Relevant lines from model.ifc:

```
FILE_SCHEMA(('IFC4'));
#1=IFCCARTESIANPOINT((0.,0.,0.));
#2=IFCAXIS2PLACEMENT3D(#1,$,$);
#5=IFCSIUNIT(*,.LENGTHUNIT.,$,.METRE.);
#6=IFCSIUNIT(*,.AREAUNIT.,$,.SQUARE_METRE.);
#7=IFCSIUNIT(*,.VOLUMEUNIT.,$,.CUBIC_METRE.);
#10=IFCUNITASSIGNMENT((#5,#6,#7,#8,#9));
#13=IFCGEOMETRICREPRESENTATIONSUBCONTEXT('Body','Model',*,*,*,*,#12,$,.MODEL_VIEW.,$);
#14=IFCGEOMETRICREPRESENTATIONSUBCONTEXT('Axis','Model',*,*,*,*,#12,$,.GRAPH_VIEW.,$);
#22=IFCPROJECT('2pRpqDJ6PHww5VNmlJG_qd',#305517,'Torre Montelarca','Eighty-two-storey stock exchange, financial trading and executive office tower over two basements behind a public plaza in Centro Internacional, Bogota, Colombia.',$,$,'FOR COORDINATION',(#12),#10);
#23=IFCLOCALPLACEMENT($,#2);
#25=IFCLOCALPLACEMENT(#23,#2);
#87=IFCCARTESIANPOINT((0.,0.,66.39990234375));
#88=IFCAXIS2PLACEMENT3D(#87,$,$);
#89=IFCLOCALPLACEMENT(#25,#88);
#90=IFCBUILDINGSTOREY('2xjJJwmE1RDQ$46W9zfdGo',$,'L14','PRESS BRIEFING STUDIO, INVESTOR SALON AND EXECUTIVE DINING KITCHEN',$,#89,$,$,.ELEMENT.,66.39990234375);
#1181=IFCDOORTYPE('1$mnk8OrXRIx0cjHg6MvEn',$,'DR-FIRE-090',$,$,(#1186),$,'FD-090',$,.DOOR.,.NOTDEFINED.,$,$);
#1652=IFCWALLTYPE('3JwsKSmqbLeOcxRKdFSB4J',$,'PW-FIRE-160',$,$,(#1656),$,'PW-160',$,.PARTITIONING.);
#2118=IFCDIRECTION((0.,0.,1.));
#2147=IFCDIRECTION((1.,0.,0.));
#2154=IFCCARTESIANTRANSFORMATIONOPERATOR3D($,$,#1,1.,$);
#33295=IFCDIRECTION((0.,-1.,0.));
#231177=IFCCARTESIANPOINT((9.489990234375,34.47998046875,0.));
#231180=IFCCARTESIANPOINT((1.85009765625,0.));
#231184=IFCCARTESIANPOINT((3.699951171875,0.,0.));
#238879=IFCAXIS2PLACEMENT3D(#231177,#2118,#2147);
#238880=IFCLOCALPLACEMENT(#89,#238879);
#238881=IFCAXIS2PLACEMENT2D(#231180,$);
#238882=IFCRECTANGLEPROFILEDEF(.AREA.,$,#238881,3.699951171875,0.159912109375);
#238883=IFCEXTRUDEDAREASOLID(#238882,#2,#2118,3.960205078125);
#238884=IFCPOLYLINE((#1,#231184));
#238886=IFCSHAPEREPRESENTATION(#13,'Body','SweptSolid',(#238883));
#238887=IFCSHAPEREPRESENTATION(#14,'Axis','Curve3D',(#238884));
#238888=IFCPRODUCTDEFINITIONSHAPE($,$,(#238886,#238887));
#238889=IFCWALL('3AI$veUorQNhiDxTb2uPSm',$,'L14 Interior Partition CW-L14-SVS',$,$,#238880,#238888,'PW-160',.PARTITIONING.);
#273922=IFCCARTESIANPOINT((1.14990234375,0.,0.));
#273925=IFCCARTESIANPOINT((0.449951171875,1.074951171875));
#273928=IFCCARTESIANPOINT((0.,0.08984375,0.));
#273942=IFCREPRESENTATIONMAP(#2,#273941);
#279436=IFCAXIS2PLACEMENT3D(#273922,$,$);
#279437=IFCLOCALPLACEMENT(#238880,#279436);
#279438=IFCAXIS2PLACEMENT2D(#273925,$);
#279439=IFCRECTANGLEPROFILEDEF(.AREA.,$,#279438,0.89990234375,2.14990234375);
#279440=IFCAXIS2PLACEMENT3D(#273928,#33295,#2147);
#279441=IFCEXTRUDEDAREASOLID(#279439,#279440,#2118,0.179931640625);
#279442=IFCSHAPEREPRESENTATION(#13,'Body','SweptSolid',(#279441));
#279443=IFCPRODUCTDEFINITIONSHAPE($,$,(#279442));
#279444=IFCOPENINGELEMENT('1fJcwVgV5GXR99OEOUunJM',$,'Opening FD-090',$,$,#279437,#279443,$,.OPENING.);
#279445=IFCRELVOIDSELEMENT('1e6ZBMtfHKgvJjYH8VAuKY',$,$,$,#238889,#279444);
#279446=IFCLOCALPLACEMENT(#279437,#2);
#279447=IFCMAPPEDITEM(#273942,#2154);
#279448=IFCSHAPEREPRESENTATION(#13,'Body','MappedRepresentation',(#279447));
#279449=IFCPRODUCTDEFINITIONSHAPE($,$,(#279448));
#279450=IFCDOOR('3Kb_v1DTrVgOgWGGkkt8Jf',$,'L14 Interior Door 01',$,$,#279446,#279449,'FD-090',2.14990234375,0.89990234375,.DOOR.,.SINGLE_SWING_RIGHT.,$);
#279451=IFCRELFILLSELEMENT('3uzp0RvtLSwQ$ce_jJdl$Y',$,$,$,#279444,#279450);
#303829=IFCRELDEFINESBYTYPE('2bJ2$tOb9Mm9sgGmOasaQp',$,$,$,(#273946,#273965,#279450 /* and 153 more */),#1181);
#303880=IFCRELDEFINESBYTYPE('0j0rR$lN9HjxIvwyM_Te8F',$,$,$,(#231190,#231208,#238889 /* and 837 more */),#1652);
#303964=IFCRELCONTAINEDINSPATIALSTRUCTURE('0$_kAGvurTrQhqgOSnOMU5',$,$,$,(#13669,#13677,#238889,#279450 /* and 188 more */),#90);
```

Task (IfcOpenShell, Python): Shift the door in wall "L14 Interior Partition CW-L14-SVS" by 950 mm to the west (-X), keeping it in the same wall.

```python
import ifcopenshell
import ifcopenshell.api.geometry
import ifcopenshell.util.placement

model = ifcopenshell.open("model.ifc")

door = model.by_guid("3Kb_v1DTrVgOgWGGkkt8Jf")
opening = door.FillsVoids[0].RelatingOpeningElement
wall = opening.VoidsElements[0].RelatingBuildingElement

wall_matrix = ifcopenshell.util.placement.get_local_placement(wall.ObjectPlacement)
shift = wall_matrix[:3, 0] * -0.95
before = ifcopenshell.util.placement.get_local_placement(door.ObjectPlacement)[:3, 3].copy()

# The door is placed relative to its opening, so it follows when the opening moves.
matrix = ifcopenshell.util.placement.get_local_placement(opening.ObjectPlacement)
matrix[:3, 3] += shift
ifcopenshell.api.geometry.edit_object_placement(
    model, product=opening, matrix=matrix, is_si=False, should_transform_children=True
)

after = ifcopenshell.util.placement.get_local_placement(door.ObjectPlacement)[:3, 3]
print("door moved by", (after - before).round(3) + 0.0)

model.write("model_rev.ifc")
```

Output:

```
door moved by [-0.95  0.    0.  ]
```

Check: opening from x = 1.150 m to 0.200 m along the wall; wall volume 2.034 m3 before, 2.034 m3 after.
